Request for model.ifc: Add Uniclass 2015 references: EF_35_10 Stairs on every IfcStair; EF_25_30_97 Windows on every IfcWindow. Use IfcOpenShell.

First a look at what the model holds.

```python
import ifcopenshell

model = ifcopenshell.open("model.ifc")
print(model.schema)
print("classifications:", [c.Name for c in model.by_type("IfcClassification")])
for ifc_class in ("IfcDoor", "IfcRoof", "IfcStair", "IfcWall", "IfcWindow"):
    print(ifc_class, len(model.by_type(ifc_class)))
```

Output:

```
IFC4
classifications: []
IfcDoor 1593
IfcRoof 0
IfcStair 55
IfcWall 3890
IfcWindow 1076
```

```python
import ifcopenshell
import ifcopenshell.api.classification

model = ifcopenshell.open("model.ifc")

system = ifcopenshell.api.classification.add_classification(model, classification="Uniclass 2015")

codes = {
    "IfcStair": ("EF_35_10", "Stairs"),
    "IfcWindow": ("EF_25_30_97", "Windows"),
}
for ifc_class, (code, name) in codes.items():
    products = model.by_type(ifc_class)
    ifcopenshell.api.classification.add_reference(
        model, products=products, classification=system, identification=code, name=name
    )
    print(code, len(products))

model.write("model_updated.ifc")
```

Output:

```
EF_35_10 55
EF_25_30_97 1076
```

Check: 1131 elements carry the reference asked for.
